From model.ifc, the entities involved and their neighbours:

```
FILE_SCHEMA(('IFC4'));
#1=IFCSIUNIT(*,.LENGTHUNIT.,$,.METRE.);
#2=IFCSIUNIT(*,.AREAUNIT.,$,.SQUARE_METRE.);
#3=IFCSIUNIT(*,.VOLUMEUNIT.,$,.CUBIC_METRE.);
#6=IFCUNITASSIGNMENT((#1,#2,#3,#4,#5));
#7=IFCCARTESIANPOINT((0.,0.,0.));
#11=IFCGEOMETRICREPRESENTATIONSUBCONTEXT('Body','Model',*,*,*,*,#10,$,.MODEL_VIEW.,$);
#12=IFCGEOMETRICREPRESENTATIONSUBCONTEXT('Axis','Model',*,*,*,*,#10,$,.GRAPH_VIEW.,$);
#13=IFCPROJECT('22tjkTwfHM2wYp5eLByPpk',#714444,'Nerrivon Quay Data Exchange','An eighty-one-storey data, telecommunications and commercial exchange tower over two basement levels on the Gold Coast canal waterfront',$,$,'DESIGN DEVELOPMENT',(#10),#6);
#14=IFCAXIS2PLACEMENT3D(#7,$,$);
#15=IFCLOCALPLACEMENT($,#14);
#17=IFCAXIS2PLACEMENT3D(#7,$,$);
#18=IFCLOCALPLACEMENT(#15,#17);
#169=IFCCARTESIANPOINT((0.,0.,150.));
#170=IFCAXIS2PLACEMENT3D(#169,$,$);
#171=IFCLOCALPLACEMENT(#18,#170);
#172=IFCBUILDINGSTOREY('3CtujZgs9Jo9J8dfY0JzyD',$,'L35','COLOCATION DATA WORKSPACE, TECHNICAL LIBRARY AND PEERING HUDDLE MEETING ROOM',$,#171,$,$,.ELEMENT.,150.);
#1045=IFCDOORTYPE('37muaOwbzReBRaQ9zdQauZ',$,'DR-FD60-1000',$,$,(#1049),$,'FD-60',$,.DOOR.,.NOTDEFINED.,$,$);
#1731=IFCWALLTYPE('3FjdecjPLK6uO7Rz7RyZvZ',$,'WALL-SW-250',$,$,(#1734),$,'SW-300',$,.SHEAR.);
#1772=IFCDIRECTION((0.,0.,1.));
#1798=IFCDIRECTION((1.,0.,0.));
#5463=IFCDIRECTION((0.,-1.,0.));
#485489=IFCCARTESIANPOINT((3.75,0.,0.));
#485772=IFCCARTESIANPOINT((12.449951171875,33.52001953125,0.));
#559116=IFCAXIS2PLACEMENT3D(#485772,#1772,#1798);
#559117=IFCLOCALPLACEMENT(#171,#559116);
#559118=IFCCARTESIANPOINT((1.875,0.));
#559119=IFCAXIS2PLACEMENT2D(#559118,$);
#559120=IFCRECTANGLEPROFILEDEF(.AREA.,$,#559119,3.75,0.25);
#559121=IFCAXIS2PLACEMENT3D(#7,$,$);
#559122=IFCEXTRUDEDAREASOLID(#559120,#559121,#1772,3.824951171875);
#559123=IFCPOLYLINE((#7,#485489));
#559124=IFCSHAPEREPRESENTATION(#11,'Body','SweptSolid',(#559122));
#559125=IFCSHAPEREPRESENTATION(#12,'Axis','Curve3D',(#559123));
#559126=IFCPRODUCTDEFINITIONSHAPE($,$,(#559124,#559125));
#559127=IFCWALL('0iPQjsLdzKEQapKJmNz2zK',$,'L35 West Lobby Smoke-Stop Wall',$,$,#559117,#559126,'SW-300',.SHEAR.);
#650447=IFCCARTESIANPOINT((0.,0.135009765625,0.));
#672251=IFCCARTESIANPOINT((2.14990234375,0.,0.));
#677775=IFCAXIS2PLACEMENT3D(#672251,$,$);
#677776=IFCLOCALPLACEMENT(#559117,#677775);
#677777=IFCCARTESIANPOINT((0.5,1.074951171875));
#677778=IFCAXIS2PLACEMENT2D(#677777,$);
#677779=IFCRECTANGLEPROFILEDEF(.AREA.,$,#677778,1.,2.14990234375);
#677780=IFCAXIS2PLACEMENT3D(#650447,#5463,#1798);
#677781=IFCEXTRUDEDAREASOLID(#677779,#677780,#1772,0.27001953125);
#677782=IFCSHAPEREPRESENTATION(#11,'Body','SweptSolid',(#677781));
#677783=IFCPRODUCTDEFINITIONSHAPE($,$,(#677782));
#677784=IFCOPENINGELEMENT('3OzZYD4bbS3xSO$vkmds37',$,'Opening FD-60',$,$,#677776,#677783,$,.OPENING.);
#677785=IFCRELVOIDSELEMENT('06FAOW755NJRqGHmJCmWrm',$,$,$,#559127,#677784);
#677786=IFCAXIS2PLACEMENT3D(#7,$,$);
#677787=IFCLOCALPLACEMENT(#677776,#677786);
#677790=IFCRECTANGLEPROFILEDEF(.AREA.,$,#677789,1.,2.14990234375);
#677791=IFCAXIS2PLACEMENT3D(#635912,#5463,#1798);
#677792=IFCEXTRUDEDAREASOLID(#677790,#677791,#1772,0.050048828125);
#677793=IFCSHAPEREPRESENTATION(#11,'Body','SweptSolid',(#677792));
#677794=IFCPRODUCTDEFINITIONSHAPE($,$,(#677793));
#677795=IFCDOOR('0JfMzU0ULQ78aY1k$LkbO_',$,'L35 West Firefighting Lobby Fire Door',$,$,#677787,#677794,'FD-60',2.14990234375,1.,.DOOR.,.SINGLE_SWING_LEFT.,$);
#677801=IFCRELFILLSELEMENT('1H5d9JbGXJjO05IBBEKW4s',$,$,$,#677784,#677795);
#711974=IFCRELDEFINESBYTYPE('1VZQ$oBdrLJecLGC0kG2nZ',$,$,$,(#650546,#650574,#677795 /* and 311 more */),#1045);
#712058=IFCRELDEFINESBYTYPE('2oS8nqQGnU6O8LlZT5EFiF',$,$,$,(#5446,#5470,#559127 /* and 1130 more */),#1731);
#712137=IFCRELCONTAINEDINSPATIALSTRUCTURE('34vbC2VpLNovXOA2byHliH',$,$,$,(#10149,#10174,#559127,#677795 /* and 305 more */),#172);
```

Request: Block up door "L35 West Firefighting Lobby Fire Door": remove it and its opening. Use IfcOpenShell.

```python
import ifcopenshell
import ifcopenshell.api.feature
import ifcopenshell.api.root
import ifcopenshell.geom
import ifcopenshell.util.shape

model = ifcopenshell.open("model.ifc")
settings = ifcopenshell.geom.settings()


def volume(element):
    """Net volume in cubic metres, openings subtracted."""
    shape = ifcopenshell.geom.create_shape(settings, element)
    return ifcopenshell.util.shape.get_volume(shape.geometry)


door = model.by_id(677795)
opening = door.FillsVoids[0].RelatingOpeningElement
wall = opening.VoidsElements[0].RelatingBuildingElement
before = volume(wall)

ifcopenshell.api.root.remove_product(model, product=door)
ifcopenshell.api.feature.remove_feature(model, feature=opening)

after = volume(wall)

print(f"wall volume {before:.3f} -> {after:.3f} m3")

model.write("model-out.ifc")
```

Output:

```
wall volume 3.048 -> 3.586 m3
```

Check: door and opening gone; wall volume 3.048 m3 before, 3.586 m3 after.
